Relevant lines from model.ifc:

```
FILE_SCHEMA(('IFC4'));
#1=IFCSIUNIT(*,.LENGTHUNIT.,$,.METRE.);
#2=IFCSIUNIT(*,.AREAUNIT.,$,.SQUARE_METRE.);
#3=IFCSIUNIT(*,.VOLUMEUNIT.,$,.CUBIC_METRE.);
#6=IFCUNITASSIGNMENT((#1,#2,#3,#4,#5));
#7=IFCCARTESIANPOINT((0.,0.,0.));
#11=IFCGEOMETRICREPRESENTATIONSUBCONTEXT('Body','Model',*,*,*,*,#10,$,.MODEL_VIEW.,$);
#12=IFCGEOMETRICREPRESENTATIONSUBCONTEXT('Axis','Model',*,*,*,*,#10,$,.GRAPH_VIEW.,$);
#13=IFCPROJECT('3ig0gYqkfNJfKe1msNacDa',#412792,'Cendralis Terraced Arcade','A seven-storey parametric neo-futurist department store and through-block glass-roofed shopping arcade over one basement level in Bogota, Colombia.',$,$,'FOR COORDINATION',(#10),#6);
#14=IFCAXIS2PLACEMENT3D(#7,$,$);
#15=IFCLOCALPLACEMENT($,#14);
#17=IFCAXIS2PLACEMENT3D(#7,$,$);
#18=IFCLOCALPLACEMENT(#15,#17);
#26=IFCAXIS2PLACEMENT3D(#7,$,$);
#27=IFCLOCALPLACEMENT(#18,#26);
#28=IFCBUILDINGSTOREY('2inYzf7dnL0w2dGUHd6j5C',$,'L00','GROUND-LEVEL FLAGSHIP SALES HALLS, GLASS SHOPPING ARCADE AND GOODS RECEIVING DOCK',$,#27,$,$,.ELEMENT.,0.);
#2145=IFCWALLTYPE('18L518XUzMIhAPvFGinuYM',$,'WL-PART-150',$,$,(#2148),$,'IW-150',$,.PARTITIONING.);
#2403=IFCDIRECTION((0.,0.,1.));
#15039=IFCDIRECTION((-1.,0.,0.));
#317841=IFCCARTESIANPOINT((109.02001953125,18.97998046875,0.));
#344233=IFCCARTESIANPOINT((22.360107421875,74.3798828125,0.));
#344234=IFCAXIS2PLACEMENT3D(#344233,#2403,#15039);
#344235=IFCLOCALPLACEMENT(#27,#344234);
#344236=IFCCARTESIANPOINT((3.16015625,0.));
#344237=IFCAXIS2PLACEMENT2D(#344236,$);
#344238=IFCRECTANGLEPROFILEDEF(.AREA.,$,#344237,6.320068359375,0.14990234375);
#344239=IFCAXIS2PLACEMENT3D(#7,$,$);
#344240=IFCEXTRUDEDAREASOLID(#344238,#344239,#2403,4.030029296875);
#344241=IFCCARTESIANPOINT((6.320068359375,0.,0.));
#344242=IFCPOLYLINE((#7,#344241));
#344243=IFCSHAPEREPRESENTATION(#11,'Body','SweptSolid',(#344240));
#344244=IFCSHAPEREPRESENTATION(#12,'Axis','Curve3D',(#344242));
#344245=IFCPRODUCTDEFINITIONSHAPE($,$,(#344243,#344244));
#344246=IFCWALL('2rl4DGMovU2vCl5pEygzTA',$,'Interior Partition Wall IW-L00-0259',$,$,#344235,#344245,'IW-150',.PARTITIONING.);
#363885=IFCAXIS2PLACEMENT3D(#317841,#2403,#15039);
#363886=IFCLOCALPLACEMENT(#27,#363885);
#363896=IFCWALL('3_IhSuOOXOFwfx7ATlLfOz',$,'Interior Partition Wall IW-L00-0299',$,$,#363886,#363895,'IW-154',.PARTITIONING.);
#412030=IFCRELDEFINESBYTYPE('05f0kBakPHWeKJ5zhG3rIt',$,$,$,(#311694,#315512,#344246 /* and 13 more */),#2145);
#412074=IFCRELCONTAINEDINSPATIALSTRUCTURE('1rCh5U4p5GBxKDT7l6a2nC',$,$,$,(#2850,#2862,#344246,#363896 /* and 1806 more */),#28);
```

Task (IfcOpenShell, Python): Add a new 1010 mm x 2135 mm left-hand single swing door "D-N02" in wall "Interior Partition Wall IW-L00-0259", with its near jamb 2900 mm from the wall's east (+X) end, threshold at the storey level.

```python
import numpy as np
import ifcopenshell
import ifcopenshell.api.feature
import ifcopenshell.api.geometry
import ifcopenshell.api.root
import ifcopenshell.api.spatial
import ifcopenshell.geom
import ifcopenshell.util.element
import ifcopenshell.util.placement
import ifcopenshell.util.representation
import ifcopenshell.util.shape
import ifcopenshell.util.unit

model = ifcopenshell.open("model.ifc")
unit_scale = ifcopenshell.util.unit.calculate_unit_scale(model)
settings = ifcopenshell.geom.settings()


def volume(element):
    """Net volume in cubic metres, openings subtracted."""
    shape = ifcopenshell.geom.create_shape(settings, element)
    return ifcopenshell.util.shape.get_volume(shape.geometry)


wall = model.by_guid("2rl4DGMovU2vCl5pEygzTA")
storey = ifcopenshell.util.element.get_container(wall, ifc_class="IfcBuildingStorey")
context = ifcopenshell.util.representation.get_context(model, "Model", "Body", "MODEL_VIEW")
before = volume(wall)

width, height, from_end, sill = 1.01, 2.135, 2.9, 0.0  # metres

# The wall runs along its own X axis, and the end named is its -X end.
wall_shape = ifcopenshell.geom.create_shape(settings, wall)
x, y, z = ifcopenshell.util.shape.get_vertices(wall_shape.geometry).T
start = x.min() + from_end
face, thickness = float(y.min()), float(y.max() - y.min())
wall_matrix = ifcopenshell.util.placement.get_local_placement(wall.ObjectPlacement)
level = ifcopenshell.util.placement.get_local_placement(storey.ObjectPlacement)[2, 3]


def in_wall(x, y):
    """Placement at x, y metres in the wall's axes, at sill height."""
    matrix = wall_matrix.copy()
    matrix[:, 3] = wall_matrix @ np.array([x / unit_scale, y / unit_scale, 0.0, 1.0])
    matrix[2, 3] = level + sill / unit_scale
    return matrix


# Opening: a box that overshoots both wall faces by 50 mm.
opening = ifcopenshell.api.root.create_entity(model, ifc_class="IfcOpeningElement", predefined_type="OPENING")
box = ifcopenshell.api.geometry.add_wall_representation(
    model, context=context, length=width, height=height, thickness=thickness + 0.1
)
ifcopenshell.api.geometry.assign_representation(model, product=opening, representation=box)
ifcopenshell.api.geometry.edit_object_placement(model, product=opening, matrix=in_wall(start, face - 0.05), is_si=False)
ifcopenshell.api.feature.add_feature(model, feature=opening, element=wall)

door = ifcopenshell.api.root.create_entity(model, ifc_class="IfcDoor", name="D-N02", predefined_type="DOOR")
door.OverallWidth, door.OverallHeight = width / unit_scale, height / unit_scale
door.OperationType = "SINGLE_SWING_LEFT"
body = ifcopenshell.api.geometry.add_door_representation(
    model,
    context=context,
    overall_width=door.OverallWidth,
    overall_height=door.OverallHeight,
    operation_type="SINGLE_SWING_LEFT",
    lining_properties={"LiningDepth": thickness / unit_scale, "ThresholdDepth": thickness / unit_scale},
)
ifcopenshell.api.geometry.assign_representation(model, product=door, representation=body)
ifcopenshell.api.spatial.assign_container(model, products=[door], relating_structure=storey)
ifcopenshell.api.feature.add_filling(model, opening=opening, element=door)

# The lining spans the wall, so the door starts at the wall face.
ifcopenshell.api.geometry.edit_object_placement(model, product=door, matrix=in_wall(start, face), is_si=False)

after = volume(wall)

print(f"wall volume {before:.3f} -> {after:.3f} m3")

model.write("model_rev.ifc")
```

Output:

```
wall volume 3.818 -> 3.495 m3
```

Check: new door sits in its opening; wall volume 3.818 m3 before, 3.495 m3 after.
